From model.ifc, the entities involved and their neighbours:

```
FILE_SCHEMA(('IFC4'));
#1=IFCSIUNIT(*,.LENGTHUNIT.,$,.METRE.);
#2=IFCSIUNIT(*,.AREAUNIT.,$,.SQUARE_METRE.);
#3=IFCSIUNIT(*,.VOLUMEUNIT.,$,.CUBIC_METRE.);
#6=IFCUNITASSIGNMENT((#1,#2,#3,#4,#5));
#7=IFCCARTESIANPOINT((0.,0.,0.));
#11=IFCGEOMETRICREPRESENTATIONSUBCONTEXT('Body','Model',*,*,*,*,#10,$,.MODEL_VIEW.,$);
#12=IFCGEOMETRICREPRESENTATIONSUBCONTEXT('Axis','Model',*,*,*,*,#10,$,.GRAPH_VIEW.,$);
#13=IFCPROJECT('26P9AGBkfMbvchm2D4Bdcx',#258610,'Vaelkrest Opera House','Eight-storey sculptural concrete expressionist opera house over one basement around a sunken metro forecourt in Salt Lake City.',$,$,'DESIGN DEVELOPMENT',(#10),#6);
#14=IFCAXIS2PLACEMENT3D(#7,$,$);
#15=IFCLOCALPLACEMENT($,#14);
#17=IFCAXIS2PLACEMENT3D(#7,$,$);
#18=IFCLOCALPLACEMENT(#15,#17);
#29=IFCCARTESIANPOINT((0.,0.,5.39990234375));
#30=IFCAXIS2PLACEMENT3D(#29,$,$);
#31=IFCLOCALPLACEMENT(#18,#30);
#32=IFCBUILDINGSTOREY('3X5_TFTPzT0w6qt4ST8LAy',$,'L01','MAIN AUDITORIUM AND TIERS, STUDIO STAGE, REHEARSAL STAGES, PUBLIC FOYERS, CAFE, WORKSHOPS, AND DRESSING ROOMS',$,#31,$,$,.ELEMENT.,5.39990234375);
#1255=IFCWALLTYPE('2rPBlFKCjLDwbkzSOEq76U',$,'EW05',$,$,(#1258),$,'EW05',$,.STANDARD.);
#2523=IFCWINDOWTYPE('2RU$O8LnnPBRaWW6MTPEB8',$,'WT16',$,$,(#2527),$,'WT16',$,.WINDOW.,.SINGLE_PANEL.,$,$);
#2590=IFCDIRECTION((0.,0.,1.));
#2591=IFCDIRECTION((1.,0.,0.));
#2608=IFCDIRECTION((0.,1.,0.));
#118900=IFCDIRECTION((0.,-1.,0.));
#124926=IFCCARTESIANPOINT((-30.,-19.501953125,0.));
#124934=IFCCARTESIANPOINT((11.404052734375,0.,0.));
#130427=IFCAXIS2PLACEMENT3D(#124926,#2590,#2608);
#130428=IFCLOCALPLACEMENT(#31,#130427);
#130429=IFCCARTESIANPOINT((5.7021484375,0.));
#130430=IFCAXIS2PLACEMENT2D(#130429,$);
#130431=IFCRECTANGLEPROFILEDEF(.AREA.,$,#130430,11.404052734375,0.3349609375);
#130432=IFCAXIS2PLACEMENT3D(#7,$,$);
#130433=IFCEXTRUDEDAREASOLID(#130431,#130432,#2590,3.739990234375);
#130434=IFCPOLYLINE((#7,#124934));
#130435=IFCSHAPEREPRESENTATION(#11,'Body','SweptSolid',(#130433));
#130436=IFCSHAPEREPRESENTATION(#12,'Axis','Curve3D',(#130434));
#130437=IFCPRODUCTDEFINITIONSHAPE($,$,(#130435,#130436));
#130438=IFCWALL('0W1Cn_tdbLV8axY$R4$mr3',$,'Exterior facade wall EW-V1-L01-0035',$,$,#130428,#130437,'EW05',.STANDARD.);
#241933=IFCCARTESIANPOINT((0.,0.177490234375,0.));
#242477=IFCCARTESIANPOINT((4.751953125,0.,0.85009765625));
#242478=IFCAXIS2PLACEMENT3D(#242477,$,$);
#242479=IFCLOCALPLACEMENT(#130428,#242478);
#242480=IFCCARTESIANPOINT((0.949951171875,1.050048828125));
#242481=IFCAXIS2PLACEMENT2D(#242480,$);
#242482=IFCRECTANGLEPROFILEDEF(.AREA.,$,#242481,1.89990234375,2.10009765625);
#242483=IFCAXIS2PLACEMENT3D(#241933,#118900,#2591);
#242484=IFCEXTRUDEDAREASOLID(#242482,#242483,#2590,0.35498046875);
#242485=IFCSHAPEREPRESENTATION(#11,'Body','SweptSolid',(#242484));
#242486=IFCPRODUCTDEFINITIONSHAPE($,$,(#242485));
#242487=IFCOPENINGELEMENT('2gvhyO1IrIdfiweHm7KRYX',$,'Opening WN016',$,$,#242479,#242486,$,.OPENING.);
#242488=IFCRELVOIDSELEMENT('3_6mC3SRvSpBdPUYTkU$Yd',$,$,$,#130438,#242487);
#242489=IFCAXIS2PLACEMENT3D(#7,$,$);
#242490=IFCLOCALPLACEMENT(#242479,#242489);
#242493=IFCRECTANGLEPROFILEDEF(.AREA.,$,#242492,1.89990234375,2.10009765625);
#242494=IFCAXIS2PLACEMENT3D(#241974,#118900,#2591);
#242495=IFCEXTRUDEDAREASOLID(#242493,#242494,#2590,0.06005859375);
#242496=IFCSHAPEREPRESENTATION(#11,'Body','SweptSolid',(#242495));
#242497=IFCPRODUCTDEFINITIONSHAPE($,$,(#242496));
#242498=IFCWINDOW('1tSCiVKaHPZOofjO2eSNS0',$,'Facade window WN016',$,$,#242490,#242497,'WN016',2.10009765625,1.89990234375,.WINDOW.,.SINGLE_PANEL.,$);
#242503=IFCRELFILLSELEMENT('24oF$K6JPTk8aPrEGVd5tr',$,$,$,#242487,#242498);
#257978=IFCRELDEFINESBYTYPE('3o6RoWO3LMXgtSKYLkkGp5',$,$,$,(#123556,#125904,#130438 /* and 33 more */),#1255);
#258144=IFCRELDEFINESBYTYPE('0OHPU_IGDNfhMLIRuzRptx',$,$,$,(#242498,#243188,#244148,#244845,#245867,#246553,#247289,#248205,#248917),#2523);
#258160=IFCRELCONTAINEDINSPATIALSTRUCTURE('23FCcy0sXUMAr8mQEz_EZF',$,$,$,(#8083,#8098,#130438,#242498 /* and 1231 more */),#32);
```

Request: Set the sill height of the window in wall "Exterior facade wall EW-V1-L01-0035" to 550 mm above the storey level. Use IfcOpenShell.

```python
import numpy as np
import ifcopenshell
import ifcopenshell.api.geometry
import ifcopenshell.geom
import ifcopenshell.util.element
import ifcopenshell.util.placement
import ifcopenshell.util.shape
import ifcopenshell.util.unit

model = ifcopenshell.open("model.ifc")
unit_scale = ifcopenshell.util.unit.calculate_unit_scale(model)

window = model.by_guid("1tSCiVKaHPZOofjO2eSNS0")
opening = window.FillsVoids[0].RelatingOpeningElement
storey = ifcopenshell.util.element.get_container(window, ifc_class="IfcBuildingStorey")
level = ifcopenshell.util.placement.get_local_placement(storey.ObjectPlacement)[2, 3]

# The opening's origin need not be at the sill, so measure its lowest point.
shape = ifcopenshell.geom.create_shape(ifcopenshell.geom.settings(), opening)
bottom = ifcopenshell.util.shape.get_shape_bottom_elevation(shape, shape.geometry) / unit_scale
dz = level + 0.55 / unit_scale - bottom

shift = np.array([0.0, 0.0, dz])
# The window is placed relative to its opening, so it follows when the opening moves.
matrix = ifcopenshell.util.placement.get_local_placement(opening.ObjectPlacement)
matrix[:3, 3] += shift
ifcopenshell.api.geometry.edit_object_placement(
    model, product=opening, matrix=matrix, is_si=False, should_transform_children=True
)

print(f"moved by {dz * unit_scale:+.3f} m")

model.write("model_rev.ifc")
```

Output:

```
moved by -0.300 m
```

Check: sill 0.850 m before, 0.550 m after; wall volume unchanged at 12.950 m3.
